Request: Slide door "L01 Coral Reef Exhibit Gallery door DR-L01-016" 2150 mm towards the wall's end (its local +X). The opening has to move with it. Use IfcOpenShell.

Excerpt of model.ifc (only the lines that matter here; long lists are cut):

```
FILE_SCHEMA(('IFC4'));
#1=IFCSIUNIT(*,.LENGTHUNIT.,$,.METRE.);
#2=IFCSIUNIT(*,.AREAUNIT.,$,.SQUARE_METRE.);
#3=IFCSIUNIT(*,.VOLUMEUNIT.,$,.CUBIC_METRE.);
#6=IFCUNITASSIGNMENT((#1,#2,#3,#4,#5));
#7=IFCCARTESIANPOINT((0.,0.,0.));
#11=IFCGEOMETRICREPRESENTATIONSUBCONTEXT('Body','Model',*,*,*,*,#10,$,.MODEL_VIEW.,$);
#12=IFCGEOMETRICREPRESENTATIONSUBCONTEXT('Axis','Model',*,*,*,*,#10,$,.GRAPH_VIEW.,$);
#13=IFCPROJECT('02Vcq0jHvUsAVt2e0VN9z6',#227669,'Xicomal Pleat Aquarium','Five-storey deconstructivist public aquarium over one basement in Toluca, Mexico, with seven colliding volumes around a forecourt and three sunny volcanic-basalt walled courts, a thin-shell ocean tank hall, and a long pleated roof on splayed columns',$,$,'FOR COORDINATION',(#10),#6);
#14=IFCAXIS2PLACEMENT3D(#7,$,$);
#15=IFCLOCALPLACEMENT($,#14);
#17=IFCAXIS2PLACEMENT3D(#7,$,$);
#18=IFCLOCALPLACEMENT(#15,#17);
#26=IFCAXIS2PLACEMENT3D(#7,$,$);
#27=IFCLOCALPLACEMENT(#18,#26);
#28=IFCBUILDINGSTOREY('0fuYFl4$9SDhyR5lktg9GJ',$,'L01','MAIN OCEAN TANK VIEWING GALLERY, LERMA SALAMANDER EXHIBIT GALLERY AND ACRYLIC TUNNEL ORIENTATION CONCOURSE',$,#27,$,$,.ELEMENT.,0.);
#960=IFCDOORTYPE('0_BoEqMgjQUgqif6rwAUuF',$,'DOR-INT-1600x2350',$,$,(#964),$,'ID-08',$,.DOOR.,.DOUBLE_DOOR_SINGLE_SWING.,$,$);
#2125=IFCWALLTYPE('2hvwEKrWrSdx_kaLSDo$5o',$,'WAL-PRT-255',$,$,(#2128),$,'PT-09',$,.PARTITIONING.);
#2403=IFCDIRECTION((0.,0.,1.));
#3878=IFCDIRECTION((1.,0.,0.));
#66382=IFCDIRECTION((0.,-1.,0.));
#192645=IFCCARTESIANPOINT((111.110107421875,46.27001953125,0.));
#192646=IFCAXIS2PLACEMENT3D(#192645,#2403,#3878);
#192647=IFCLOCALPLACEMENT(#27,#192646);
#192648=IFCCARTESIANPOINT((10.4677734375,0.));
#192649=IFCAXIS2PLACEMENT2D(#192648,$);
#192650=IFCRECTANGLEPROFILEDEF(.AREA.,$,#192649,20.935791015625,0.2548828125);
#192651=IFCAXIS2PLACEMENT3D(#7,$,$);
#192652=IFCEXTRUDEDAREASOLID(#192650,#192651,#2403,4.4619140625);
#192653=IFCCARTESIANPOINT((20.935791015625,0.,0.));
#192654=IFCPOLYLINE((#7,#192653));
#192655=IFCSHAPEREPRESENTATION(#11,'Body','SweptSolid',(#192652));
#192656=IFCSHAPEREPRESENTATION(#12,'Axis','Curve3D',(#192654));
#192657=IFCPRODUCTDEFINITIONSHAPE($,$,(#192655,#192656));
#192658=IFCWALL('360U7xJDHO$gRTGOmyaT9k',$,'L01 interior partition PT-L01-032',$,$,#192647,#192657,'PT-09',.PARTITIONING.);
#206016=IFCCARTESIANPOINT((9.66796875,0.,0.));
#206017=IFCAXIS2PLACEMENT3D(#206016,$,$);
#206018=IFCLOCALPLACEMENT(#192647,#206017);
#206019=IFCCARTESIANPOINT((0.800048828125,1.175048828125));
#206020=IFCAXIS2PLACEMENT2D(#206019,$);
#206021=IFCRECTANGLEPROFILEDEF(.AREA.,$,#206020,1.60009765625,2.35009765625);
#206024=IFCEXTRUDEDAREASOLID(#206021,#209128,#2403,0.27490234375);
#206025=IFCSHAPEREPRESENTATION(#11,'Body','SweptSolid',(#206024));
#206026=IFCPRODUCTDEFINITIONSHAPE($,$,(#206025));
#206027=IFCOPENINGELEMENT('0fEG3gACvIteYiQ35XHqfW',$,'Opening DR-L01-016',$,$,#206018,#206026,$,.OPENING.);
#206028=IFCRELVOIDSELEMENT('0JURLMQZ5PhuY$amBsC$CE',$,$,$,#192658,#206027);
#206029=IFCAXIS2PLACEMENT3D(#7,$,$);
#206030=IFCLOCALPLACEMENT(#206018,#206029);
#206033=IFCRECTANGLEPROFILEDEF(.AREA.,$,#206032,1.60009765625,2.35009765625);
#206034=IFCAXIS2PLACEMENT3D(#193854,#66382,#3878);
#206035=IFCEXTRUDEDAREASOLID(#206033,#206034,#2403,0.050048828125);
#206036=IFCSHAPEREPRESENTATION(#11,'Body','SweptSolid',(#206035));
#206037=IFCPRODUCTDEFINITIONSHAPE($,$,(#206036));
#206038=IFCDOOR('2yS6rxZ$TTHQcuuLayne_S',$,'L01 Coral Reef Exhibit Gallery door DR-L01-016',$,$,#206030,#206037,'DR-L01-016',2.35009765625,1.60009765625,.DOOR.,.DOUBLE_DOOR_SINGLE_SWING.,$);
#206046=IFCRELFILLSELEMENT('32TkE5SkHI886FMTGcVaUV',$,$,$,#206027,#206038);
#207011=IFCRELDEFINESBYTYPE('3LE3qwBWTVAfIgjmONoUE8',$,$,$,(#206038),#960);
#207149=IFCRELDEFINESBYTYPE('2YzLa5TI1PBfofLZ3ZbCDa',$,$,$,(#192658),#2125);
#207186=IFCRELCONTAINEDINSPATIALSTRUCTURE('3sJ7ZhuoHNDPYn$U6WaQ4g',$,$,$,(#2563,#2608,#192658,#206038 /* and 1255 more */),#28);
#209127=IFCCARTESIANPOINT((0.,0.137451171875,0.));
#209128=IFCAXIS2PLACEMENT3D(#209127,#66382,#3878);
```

```python
import ifcopenshell
import ifcopenshell.api.geometry
import ifcopenshell.util.placement
import ifcopenshell.util.unit

model = ifcopenshell.open("model.ifc")
unit_scale = ifcopenshell.util.unit.calculate_unit_scale(model)

door = model.by_guid("2yS6rxZ$TTHQcuuLayne_S")
opening = door.FillsVoids[0].RelatingOpeningElement
wall = opening.VoidsElements[0].RelatingBuildingElement

wall_matrix = ifcopenshell.util.placement.get_local_placement(wall.ObjectPlacement)
shift = wall_matrix[:3, 0] * 2.15 / unit_scale
before = ifcopenshell.util.placement.get_local_placement(door.ObjectPlacement)[:3, 3].copy()

# The door is placed relative to its opening, so it follows when the opening moves.
matrix = ifcopenshell.util.placement.get_local_placement(opening.ObjectPlacement)
matrix[:3, 3] += shift
ifcopenshell.api.geometry.edit_object_placement(
    model, product=opening, matrix=matrix, is_si=False, should_transform_children=True
)

after = ifcopenshell.util.placement.get_local_placement(door.ObjectPlacement)[:3, 3]
print("door moved by", (after - before).round(3) + 0.0)

model.write("model_edited.ifc")
```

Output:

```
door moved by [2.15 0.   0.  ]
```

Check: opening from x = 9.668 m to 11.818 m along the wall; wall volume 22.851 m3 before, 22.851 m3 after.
